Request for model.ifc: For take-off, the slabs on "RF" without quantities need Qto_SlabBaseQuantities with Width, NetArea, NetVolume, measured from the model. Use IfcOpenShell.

First a look at what the model holds.

```python
import ifcopenshell
import ifcopenshell.util.element
import ifcopenshell.util.unit

model = ifcopenshell.open("model.ifc")
print(model.schema)
for unit_type in ("LENGTHUNIT", "AREAUNIT", "VOLUMEUNIT"):
    print(unit_type, ifcopenshell.util.unit.calculate_unit_scale(model, unit_type))
storey = next(s for s in model.by_type("IfcBuildingStorey") if s.Name == "RF")
slabs = [e for e in ifcopenshell.util.element.get_decomposition(storey) if e.is_a("IfcSlab")]
for e in sorted(slabs, key=lambda e: e.id()):
    print(e.id(), e.is_a(), e.Name, list(ifcopenshell.util.element.get_psets(e, qtos_only=True)), sep=" | ")
```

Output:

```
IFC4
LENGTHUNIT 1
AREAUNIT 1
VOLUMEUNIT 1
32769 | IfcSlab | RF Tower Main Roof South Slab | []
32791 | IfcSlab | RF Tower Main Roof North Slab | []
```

```python
import ifcopenshell
import ifcopenshell.api.pset
import ifcopenshell.geom
import ifcopenshell.util.element
import ifcopenshell.util.shape
import ifcopenshell.util.unit

model = ifcopenshell.open("model.ifc")
unit_scale = ifcopenshell.util.unit.calculate_unit_scale(model)
area_scale = ifcopenshell.util.unit.calculate_unit_scale(model, "AREAUNIT")
volume_scale = ifcopenshell.util.unit.calculate_unit_scale(model, "VOLUMEUNIT")
settings = ifcopenshell.geom.settings()

storey = next(s for s in model.by_type("IfcBuildingStorey") if s.Name == "RF")
slabs = [e for e in ifcopenshell.util.element.get_decomposition(storey) if e.is_a("IfcSlab")]

for e in sorted(slabs, key=lambda e: e.id()):
    if ifcopenshell.util.element.get_psets(e, qtos_only=True, should_inherit=False):
        continue
    # Geometry comes back in metres, in the element's own axes.
    shape = ifcopenshell.geom.create_shape(settings, e)
    values = {
        "Width": ifcopenshell.util.shape.get_z(shape.geometry) / unit_scale,
        "NetArea": ifcopenshell.util.shape.get_footprint_area(shape.geometry) / area_scale,
        "NetVolume": ifcopenshell.util.shape.get_volume(shape.geometry) / volume_scale,
    }
    qto = ifcopenshell.api.pset.add_qto(model, product=e, name="Qto_SlabBaseQuantities")
    ifcopenshell.api.pset.edit_qto(model, qto=qto, properties=values)
    print(e.id(), {k: round(v, 3) for k, v in values.items()})

model.write("model_rev.ifc")
```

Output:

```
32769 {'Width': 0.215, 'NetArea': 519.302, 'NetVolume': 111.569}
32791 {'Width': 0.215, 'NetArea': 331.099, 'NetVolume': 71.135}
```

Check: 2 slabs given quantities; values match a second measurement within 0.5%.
